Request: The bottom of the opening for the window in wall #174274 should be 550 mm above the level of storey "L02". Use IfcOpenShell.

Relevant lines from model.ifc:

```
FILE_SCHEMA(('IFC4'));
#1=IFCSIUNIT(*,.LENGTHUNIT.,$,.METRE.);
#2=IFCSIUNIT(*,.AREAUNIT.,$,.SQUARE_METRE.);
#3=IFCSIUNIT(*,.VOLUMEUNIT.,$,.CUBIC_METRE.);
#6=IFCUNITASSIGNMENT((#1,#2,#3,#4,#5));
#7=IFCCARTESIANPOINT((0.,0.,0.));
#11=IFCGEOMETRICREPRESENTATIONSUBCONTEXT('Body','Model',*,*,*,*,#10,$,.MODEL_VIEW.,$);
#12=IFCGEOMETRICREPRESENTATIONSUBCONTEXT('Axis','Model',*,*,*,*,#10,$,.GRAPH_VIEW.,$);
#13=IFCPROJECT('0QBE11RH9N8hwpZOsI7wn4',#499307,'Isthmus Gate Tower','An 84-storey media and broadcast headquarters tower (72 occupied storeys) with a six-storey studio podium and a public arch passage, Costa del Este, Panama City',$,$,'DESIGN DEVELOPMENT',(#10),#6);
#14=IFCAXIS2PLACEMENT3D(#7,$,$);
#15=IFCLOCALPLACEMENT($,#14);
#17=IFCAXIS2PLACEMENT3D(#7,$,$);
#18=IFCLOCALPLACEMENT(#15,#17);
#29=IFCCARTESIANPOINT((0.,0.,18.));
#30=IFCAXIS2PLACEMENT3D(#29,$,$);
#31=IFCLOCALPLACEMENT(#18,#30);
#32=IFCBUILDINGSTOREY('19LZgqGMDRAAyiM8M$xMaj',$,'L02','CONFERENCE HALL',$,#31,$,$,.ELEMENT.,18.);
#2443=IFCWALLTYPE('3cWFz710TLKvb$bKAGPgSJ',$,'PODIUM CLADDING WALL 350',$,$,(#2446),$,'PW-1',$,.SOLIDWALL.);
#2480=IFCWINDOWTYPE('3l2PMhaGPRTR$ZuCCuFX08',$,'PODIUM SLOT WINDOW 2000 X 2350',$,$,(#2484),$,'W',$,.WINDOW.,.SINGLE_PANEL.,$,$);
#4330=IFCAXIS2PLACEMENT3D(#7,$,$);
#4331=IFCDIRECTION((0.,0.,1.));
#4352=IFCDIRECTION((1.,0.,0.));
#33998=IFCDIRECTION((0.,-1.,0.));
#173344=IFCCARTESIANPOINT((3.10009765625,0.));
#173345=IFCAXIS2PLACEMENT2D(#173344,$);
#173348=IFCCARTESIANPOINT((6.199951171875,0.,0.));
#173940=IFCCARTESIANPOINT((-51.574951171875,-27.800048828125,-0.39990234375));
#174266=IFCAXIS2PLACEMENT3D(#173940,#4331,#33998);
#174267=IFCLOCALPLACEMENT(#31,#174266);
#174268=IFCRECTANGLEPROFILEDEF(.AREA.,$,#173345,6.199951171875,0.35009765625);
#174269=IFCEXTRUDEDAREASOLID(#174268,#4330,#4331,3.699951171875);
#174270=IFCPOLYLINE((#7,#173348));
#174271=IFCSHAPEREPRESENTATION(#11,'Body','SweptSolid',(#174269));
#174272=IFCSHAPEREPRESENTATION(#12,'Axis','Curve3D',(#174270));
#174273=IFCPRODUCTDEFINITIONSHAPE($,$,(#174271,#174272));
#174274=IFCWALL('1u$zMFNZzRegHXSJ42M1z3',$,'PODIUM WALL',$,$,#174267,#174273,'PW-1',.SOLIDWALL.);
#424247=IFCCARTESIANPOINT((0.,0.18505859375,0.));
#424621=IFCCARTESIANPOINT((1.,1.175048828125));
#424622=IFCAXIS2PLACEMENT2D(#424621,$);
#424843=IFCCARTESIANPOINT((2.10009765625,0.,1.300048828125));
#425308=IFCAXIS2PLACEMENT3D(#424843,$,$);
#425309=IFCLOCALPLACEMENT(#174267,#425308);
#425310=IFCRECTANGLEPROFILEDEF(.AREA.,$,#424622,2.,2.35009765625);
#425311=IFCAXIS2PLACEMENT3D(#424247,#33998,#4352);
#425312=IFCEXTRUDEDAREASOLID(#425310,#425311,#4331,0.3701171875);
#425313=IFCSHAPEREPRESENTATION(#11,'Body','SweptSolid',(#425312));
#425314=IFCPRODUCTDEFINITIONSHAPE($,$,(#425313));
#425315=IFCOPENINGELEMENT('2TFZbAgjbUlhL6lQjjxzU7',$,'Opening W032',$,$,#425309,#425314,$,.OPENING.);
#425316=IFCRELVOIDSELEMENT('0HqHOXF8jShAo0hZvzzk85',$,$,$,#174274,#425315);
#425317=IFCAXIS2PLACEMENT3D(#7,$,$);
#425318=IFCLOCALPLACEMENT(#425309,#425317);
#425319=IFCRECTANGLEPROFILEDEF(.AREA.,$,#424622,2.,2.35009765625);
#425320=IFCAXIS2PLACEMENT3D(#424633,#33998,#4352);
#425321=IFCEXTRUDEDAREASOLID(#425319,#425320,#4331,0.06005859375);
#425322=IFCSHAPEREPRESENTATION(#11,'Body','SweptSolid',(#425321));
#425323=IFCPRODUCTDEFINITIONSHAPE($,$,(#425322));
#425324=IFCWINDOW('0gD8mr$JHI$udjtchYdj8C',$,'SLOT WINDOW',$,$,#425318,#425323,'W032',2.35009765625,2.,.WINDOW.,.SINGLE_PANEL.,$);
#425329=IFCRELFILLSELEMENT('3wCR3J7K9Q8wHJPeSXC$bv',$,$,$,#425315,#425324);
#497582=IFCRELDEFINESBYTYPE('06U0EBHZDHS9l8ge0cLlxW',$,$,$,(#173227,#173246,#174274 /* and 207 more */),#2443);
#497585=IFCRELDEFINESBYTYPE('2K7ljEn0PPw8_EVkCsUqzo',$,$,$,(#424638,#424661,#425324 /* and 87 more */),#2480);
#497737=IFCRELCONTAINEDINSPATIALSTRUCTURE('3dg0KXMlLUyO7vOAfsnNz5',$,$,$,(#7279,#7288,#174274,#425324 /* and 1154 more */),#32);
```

```python
import numpy as np
import ifcopenshell
import ifcopenshell.api.geometry
import ifcopenshell.geom
import ifcopenshell.util.element
import ifcopenshell.util.placement
import ifcopenshell.util.shape
import ifcopenshell.util.unit

model = ifcopenshell.open("model.ifc")
unit_scale = ifcopenshell.util.unit.calculate_unit_scale(model)

window = model.by_id(425324)
opening = window.FillsVoids[0].RelatingOpeningElement
storey = ifcopenshell.util.element.get_container(window, ifc_class="IfcBuildingStorey")
level = ifcopenshell.util.placement.get_local_placement(storey.ObjectPlacement)[2, 3]

# The opening's origin need not be at the sill, so measure its lowest point.
shape = ifcopenshell.geom.create_shape(ifcopenshell.geom.settings(), opening)
bottom = ifcopenshell.util.shape.get_shape_bottom_elevation(shape, shape.geometry) / unit_scale
dz = level + 0.55 / unit_scale - bottom

shift = np.array([0.0, 0.0, dz])
# The window is placed relative to its opening, so it follows when the opening moves.
matrix = ifcopenshell.util.placement.get_local_placement(opening.ObjectPlacement)
matrix[:3, 3] += shift
ifcopenshell.api.geometry.edit_object_placement(
    model, product=opening, matrix=matrix, is_si=False, should_transform_children=True
)

print(f"moved by {dz * unit_scale:+.3f} m")

model.write("model-out.ifc")
```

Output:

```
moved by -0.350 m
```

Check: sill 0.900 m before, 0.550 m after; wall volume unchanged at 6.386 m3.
